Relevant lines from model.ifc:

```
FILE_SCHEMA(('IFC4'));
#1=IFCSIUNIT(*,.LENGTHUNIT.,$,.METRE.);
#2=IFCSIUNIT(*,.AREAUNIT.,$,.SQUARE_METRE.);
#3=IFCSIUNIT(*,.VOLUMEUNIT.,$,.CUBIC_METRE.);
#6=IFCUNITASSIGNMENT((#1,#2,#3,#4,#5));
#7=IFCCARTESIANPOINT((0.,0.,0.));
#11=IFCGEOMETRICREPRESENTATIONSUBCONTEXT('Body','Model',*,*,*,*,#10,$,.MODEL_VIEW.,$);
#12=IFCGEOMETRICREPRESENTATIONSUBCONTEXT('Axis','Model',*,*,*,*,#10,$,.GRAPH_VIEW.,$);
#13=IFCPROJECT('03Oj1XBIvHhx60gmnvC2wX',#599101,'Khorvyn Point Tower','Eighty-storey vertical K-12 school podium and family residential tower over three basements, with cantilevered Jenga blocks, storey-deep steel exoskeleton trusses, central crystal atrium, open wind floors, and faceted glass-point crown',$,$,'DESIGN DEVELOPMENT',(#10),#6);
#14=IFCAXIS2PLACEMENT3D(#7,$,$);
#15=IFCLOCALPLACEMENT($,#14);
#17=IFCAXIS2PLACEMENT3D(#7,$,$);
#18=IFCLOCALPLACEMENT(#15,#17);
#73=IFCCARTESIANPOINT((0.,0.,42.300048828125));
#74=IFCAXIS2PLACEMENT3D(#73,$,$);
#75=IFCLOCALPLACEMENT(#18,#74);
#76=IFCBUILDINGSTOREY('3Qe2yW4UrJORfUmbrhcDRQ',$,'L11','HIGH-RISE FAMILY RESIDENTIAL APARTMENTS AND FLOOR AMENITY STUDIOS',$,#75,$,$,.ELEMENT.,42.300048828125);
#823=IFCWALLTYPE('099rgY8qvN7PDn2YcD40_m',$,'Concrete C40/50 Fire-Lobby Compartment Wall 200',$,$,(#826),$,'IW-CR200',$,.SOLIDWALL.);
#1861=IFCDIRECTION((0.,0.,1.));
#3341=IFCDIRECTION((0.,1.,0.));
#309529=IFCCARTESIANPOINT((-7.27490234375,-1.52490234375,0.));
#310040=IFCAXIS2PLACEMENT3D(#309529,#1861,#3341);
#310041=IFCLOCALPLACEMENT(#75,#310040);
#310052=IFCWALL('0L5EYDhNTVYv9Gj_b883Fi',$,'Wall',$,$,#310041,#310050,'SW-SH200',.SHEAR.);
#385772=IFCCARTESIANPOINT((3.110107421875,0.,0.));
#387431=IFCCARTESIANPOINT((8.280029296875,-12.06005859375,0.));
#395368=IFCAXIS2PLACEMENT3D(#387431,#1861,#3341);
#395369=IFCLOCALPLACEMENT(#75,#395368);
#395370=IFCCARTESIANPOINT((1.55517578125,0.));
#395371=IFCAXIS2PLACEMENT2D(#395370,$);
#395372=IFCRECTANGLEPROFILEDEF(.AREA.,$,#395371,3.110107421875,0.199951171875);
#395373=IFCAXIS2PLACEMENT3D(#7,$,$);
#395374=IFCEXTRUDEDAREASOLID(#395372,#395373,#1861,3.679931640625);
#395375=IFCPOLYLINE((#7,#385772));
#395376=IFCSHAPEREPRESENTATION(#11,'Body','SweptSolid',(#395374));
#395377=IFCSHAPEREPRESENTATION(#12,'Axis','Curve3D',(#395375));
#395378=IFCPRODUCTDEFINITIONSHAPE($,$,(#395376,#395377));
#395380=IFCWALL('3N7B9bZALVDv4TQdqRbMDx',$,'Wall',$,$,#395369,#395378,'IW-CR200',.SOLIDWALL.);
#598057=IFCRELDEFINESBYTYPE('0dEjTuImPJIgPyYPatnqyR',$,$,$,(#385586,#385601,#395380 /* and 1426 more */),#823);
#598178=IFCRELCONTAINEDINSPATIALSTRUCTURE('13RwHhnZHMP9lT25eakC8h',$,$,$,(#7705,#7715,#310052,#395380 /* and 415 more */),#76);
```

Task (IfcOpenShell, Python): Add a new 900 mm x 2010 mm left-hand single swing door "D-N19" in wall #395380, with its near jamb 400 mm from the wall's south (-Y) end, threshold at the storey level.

```python
import numpy as np
import ifcopenshell
import ifcopenshell.api.feature
import ifcopenshell.api.geometry
import ifcopenshell.api.root
import ifcopenshell.api.spatial
import ifcopenshell.geom
import ifcopenshell.util.element
import ifcopenshell.util.placement
import ifcopenshell.util.representation
import ifcopenshell.util.shape
import ifcopenshell.util.unit

model = ifcopenshell.open("model.ifc")
unit_scale = ifcopenshell.util.unit.calculate_unit_scale(model)
settings = ifcopenshell.geom.settings()


def volume(element):
    """Net volume in cubic metres, openings subtracted."""
    shape = ifcopenshell.geom.create_shape(settings, element)
    return ifcopenshell.util.shape.get_volume(shape.geometry)


wall = model.by_guid("3N7B9bZALVDv4TQdqRbMDx")
storey = ifcopenshell.util.element.get_container(wall, ifc_class="IfcBuildingStorey")
context = ifcopenshell.util.representation.get_context(model, "Model", "Body", "MODEL_VIEW")
before = volume(wall)

width, height, from_end, sill = 0.9, 2.01, 0.4, 0.0  # metres

# The wall runs along its own X axis, and the end named is its -X end.
wall_shape = ifcopenshell.geom.create_shape(settings, wall)
x, y, z = ifcopenshell.util.shape.get_vertices(wall_shape.geometry).T
start = x.min() + from_end
face, thickness = float(y.min()), float(y.max() - y.min())
wall_matrix = ifcopenshell.util.placement.get_local_placement(wall.ObjectPlacement)
level = ifcopenshell.util.placement.get_local_placement(storey.ObjectPlacement)[2, 3]


def in_wall(x, y):
    """Placement at x, y metres in the wall's axes, at sill height."""
    matrix = wall_matrix.copy()
    matrix[:, 3] = wall_matrix @ np.array([x / unit_scale, y / unit_scale, 0.0, 1.0])
    matrix[2, 3] = level + sill / unit_scale
    return matrix


# Opening: a box that overshoots both wall faces by 50 mm.
opening = ifcopenshell.api.root.create_entity(model, ifc_class="IfcOpeningElement", predefined_type="OPENING")
box = ifcopenshell.api.geometry.add_wall_representation(
    model, context=context, length=width, height=height, thickness=thickness + 0.1
)
ifcopenshell.api.geometry.assign_representation(model, product=opening, representation=box)
ifcopenshell.api.geometry.edit_object_placement(model, product=opening, matrix=in_wall(start, face - 0.05), is_si=False)
ifcopenshell.api.feature.add_feature(model, feature=opening, element=wall)

door = ifcopenshell.api.root.create_entity(model, ifc_class="IfcDoor", name="D-N19", predefined_type="DOOR")
door.OverallWidth, door.OverallHeight = width / unit_scale, height / unit_scale
door.OperationType = "SINGLE_SWING_LEFT"
body = ifcopenshell.api.geometry.add_door_representation(
    model,
    context=context,
    overall_width=door.OverallWidth,
    overall_height=door.OverallHeight,
    operation_type="SINGLE_SWING_LEFT",
    lining_properties={"LiningDepth": thickness / unit_scale, "ThresholdDepth": thickness / unit_scale},
)
ifcopenshell.api.geometry.assign_representation(model, product=door, representation=body)
ifcopenshell.api.spatial.assign_container(model, products=[door], relating_structure=storey)
ifcopenshell.api.feature.add_filling(model, opening=opening, element=door)

# The lining spans the wall, so the door starts at the wall face.
ifcopenshell.api.geometry.edit_object_placement(model, product=door, matrix=in_wall(start, face), is_si=False)

after = volume(wall)

print(f"wall volume {before:.3f} -> {after:.3f} m3")

model.write("model_updated.ifc")
```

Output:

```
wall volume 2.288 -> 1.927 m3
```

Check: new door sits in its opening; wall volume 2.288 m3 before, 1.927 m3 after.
